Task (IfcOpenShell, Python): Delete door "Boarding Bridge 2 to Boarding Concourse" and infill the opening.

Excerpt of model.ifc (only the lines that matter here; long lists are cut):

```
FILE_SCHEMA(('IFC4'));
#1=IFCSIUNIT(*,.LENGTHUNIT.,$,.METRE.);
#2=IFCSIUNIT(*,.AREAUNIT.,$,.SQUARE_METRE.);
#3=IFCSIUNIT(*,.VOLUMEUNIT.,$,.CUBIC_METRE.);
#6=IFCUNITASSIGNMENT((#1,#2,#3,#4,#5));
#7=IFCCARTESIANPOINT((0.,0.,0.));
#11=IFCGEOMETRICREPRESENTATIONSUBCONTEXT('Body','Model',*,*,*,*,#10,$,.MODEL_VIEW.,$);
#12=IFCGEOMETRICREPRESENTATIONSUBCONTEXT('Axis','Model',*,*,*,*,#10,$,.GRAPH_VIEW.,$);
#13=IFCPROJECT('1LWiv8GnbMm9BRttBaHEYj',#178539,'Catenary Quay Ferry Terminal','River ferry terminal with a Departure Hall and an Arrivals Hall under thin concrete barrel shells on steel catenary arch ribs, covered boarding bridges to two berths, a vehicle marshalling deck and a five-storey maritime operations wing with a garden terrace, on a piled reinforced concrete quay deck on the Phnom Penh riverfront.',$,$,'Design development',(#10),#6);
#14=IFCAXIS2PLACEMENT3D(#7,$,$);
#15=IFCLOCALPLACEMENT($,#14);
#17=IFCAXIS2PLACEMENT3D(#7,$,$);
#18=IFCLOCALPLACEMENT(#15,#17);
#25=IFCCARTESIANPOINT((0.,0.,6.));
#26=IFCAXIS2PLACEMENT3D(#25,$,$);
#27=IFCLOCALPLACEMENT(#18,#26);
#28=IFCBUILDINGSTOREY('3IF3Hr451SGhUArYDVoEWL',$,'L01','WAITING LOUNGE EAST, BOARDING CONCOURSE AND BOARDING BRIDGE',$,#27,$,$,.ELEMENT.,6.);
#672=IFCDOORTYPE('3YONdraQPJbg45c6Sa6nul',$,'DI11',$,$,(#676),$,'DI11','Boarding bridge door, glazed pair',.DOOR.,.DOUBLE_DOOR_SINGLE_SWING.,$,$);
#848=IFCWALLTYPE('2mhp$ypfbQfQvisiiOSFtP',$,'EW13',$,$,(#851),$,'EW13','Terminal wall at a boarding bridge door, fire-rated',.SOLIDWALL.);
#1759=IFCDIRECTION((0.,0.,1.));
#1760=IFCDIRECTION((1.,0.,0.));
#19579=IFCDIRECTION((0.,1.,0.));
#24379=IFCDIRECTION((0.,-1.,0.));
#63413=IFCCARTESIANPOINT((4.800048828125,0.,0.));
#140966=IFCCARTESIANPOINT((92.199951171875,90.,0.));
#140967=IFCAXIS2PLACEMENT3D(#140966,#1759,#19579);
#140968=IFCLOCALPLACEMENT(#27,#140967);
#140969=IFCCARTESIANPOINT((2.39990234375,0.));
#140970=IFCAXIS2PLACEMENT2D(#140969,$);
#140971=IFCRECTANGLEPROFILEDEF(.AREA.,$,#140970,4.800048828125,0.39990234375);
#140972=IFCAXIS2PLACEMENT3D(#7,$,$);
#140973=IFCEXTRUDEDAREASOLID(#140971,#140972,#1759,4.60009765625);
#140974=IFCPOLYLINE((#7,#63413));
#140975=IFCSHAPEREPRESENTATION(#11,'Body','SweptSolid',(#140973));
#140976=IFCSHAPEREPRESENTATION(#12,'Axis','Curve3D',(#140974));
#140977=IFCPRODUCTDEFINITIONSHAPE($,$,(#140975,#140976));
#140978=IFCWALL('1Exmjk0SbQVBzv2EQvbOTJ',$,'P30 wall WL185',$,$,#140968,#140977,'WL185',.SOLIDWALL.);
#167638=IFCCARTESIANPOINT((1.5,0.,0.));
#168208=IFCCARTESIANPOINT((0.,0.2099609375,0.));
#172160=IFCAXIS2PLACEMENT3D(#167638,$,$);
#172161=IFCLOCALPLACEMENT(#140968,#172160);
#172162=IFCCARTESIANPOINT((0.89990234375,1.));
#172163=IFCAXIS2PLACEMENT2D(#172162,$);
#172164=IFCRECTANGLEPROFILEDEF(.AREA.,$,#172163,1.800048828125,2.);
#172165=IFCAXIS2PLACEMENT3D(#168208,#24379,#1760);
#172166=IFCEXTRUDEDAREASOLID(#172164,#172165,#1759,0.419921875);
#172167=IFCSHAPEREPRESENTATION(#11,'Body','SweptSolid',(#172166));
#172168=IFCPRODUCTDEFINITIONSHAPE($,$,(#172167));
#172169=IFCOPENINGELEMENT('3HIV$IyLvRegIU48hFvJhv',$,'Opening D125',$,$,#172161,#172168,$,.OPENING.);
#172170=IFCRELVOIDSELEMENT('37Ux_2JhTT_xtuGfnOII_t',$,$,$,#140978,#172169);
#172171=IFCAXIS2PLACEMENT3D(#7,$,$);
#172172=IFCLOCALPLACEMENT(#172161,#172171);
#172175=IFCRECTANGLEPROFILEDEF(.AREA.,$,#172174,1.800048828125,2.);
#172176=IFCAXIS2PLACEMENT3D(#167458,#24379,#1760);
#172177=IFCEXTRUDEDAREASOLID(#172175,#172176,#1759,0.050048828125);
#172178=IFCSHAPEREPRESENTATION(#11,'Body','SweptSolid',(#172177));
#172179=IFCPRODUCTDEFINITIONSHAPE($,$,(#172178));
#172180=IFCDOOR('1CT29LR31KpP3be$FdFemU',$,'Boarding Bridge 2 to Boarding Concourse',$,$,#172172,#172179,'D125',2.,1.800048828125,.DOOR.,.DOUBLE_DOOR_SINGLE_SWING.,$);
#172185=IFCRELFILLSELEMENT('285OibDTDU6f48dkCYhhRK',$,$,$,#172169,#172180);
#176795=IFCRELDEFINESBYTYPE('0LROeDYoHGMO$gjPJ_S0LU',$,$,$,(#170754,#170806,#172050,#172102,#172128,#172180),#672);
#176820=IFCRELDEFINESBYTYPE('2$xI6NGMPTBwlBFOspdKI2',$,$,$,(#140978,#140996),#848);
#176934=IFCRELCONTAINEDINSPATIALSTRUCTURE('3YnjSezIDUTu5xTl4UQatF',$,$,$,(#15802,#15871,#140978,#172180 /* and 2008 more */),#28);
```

```python
import ifcopenshell
import ifcopenshell.api.feature
import ifcopenshell.api.root
import ifcopenshell.geom
import ifcopenshell.util.shape

model = ifcopenshell.open("model.ifc")
settings = ifcopenshell.geom.settings()


def volume(element):
    """Net volume in cubic metres, openings subtracted."""
    shape = ifcopenshell.geom.create_shape(settings, element)
    return ifcopenshell.util.shape.get_volume(shape.geometry)


door = model.by_guid("1CT29LR31KpP3be$FdFemU")
opening = door.FillsVoids[0].RelatingOpeningElement
wall = opening.VoidsElements[0].RelatingBuildingElement
before = volume(wall)

ifcopenshell.api.root.remove_product(model, product=door)
ifcopenshell.api.feature.remove_feature(model, feature=opening)

after = volume(wall)

print(f"wall volume {before:.3f} -> {after:.3f} m3")

model.write("model_updated.ifc")
```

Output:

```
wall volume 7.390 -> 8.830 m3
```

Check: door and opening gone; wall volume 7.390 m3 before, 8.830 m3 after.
